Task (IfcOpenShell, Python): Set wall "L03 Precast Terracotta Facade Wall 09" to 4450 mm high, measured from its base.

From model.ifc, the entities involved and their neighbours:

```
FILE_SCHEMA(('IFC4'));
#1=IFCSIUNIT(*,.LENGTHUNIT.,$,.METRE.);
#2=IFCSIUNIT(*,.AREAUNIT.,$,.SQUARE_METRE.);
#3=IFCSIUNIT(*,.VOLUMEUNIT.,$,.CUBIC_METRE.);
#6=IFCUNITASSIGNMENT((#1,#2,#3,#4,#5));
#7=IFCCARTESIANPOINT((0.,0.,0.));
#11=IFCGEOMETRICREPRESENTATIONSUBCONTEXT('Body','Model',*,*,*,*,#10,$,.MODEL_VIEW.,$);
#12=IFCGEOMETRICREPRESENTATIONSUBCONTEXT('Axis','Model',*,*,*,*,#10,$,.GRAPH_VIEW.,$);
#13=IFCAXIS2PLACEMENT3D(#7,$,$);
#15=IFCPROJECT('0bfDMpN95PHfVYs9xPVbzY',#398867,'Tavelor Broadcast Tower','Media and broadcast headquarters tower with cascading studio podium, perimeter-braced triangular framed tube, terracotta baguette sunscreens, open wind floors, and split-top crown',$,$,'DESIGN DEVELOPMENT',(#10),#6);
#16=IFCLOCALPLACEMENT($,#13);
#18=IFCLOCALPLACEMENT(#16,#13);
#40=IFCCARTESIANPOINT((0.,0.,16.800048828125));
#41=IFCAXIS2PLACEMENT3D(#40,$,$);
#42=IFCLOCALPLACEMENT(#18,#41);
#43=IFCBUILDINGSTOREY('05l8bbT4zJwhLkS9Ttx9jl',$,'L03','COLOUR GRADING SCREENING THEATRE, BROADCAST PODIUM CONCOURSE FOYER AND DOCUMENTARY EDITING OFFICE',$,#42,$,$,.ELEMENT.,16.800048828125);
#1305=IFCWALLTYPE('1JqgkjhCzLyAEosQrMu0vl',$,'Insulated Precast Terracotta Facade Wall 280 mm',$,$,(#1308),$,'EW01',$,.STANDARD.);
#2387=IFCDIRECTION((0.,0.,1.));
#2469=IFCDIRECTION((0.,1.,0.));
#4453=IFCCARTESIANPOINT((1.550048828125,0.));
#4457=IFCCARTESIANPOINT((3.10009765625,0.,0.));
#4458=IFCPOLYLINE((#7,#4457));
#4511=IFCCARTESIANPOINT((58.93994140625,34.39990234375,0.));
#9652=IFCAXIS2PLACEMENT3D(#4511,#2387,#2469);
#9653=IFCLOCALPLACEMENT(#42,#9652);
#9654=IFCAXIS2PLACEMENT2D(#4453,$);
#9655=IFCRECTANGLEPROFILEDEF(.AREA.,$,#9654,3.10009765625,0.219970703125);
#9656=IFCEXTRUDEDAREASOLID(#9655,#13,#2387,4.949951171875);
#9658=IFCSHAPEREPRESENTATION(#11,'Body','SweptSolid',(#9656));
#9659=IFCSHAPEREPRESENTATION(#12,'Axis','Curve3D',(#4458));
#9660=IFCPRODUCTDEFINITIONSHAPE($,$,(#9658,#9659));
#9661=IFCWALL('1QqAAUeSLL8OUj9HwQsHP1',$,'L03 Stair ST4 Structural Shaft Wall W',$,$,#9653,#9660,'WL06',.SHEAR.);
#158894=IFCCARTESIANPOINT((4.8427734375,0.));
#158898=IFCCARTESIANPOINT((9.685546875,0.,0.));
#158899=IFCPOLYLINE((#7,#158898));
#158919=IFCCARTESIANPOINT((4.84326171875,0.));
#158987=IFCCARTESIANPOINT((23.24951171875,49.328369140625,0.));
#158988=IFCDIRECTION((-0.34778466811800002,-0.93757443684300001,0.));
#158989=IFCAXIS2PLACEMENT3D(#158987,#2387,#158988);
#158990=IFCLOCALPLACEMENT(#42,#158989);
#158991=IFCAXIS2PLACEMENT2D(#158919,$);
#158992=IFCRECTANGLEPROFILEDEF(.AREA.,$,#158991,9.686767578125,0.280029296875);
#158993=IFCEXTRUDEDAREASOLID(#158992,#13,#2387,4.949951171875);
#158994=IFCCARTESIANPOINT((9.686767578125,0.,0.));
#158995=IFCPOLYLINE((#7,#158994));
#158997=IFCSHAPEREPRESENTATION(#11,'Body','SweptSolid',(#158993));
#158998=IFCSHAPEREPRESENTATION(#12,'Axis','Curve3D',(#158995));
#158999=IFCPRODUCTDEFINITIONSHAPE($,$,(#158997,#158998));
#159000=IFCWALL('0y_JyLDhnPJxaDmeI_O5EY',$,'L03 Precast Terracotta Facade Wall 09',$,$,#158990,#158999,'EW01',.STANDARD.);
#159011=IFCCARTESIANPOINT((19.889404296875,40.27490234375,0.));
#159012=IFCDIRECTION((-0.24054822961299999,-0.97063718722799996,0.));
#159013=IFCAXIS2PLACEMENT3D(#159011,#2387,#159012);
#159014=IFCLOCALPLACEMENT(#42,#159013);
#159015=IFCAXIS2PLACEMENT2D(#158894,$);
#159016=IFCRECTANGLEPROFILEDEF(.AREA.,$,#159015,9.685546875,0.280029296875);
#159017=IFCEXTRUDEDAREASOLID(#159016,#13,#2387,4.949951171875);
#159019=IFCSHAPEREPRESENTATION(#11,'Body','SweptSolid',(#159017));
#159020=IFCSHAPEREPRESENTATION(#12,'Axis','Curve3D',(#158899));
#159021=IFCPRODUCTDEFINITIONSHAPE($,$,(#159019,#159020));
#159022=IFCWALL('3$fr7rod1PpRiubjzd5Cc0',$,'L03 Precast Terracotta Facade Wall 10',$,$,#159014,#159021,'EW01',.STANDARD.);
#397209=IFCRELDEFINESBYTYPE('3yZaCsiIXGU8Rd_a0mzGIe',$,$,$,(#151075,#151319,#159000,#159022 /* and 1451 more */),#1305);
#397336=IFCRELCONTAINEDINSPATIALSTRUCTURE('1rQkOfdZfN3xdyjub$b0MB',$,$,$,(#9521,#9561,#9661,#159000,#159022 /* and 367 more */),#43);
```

```python
import ifcopenshell
import ifcopenshell.geom
import ifcopenshell.util.representation
import ifcopenshell.util.shape

model = ifcopenshell.open("model.ifc")
settings = ifcopenshell.geom.settings()


def volume(element):
    """Net volume in cubic metres, openings subtracted."""
    shape = ifcopenshell.geom.create_shape(settings, element)
    return ifcopenshell.util.shape.get_volume(shape.geometry)


wall = model.by_guid("0y_JyLDhnPJxaDmeI_O5EY")
before = volume(wall)

body = ifcopenshell.util.representation.get_representation(wall, "Model", "Body")
solid = body.Items[0]
old_height = solid.Depth
solid.Depth = 4.45
after = volume(wall)

print(f"height {old_height:g} -> {solid.Depth:g}, volume {before:.3f} -> {after:.3f} m3")

model.write("model_edited.ifc")
```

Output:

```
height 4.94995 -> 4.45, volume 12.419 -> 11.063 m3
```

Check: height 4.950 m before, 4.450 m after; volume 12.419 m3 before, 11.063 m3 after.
